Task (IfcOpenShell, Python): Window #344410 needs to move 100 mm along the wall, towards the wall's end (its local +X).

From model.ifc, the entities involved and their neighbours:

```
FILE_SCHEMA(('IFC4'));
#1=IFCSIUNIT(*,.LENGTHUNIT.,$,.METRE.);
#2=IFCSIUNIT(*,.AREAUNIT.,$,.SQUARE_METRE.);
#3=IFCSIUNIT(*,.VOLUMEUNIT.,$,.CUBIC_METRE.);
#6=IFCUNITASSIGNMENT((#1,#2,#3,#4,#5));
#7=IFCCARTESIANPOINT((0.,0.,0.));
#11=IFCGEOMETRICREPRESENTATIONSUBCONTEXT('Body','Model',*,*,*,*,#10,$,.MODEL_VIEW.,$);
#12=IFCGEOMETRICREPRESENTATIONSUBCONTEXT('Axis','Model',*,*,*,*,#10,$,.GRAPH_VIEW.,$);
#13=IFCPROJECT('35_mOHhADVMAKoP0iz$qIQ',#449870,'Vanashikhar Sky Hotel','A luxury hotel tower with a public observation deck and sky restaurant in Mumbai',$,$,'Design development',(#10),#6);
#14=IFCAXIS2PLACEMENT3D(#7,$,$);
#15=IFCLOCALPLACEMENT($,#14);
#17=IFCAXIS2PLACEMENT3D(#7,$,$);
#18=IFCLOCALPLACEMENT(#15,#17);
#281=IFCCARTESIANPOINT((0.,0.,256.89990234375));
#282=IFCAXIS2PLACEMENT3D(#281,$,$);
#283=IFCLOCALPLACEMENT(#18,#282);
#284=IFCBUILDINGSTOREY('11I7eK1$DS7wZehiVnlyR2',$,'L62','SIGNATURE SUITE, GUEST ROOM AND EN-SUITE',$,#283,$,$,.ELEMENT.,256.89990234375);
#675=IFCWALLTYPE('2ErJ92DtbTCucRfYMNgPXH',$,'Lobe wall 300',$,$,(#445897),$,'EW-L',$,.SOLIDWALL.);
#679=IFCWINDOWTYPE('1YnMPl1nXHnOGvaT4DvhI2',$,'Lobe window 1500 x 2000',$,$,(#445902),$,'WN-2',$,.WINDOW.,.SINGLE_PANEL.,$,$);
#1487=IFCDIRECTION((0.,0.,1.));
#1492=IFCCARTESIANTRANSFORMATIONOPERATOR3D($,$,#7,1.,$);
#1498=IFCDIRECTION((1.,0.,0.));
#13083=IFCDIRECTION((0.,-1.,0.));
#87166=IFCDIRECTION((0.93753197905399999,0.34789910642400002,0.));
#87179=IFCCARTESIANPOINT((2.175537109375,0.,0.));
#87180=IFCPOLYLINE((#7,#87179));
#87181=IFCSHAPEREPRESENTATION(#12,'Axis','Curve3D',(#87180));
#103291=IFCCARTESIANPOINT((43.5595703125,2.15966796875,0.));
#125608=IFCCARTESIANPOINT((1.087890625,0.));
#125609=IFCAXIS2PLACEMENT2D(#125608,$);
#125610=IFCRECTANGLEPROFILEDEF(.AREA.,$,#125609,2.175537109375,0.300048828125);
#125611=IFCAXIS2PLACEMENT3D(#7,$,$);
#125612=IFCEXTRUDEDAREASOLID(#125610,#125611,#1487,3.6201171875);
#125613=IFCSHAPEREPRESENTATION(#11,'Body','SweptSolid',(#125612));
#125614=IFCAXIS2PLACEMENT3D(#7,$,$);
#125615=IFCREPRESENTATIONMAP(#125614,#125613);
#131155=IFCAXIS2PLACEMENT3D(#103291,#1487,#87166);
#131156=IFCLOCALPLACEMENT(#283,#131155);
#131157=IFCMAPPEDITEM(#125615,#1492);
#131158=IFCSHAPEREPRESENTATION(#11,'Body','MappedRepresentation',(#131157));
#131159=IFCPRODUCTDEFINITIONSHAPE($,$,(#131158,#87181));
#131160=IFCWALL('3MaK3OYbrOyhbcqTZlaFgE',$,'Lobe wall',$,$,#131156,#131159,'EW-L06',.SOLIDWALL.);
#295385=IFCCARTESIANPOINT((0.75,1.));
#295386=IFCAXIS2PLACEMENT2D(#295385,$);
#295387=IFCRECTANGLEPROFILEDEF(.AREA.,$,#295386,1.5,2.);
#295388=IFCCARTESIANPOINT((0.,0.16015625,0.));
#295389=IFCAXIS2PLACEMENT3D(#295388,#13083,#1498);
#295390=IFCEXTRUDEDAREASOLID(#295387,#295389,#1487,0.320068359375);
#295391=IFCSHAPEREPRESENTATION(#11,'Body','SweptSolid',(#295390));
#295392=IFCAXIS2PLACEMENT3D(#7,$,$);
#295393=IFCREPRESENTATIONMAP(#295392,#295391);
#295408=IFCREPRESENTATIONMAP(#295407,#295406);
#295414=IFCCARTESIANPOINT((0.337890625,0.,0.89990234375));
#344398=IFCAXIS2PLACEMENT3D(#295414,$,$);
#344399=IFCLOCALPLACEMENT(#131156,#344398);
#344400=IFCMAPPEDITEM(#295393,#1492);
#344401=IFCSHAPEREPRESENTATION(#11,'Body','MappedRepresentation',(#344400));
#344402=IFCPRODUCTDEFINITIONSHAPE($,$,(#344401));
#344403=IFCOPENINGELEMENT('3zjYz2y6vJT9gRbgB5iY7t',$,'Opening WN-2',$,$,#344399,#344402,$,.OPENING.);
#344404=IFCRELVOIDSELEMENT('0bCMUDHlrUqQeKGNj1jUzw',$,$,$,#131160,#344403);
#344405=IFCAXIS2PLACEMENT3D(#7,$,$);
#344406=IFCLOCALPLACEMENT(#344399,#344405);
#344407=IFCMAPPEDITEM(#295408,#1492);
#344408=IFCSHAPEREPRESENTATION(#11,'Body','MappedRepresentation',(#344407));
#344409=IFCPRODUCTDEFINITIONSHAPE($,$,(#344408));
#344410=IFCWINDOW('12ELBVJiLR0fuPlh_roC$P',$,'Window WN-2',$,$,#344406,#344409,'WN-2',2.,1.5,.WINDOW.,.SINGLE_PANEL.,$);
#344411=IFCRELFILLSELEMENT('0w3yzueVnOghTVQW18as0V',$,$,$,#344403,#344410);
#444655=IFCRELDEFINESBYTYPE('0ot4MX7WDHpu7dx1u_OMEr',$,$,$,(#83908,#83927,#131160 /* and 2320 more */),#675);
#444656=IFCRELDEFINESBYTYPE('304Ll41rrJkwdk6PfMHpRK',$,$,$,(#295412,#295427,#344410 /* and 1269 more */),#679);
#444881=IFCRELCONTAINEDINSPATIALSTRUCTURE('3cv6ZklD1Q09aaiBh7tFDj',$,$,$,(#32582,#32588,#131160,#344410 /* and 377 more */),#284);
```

```python
import ifcopenshell
import ifcopenshell.api.geometry
import ifcopenshell.util.placement
import ifcopenshell.util.unit

model = ifcopenshell.open("model.ifc")
unit_scale = ifcopenshell.util.unit.calculate_unit_scale(model)

window = model.by_id(344410)
opening = window.FillsVoids[0].RelatingOpeningElement
wall = opening.VoidsElements[0].RelatingBuildingElement

wall_matrix = ifcopenshell.util.placement.get_local_placement(wall.ObjectPlacement)
shift = wall_matrix[:3, 0] * 0.1 / unit_scale
before = ifcopenshell.util.placement.get_local_placement(window.ObjectPlacement)[:3, 3].copy()

# The window is placed relative to its opening, so it follows when the opening moves.
matrix = ifcopenshell.util.placement.get_local_placement(opening.ObjectPlacement)
matrix[:3, 3] += shift
ifcopenshell.api.geometry.edit_object_placement(
    model, product=opening, matrix=matrix, is_si=False, should_transform_children=True
)

after = ifcopenshell.util.placement.get_local_placement(window.ObjectPlacement)[:3, 3]
print("window moved by", (after - before).round(3) + 0.0)

model.write("model_rev.ifc")
```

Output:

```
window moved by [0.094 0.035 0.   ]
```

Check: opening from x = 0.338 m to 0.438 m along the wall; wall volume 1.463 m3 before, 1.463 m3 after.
